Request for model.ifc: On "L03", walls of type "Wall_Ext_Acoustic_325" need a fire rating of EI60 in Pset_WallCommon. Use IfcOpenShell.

First a look at what the model holds.

```python
import ifcopenshell
import ifcopenshell.util.element

model = ifcopenshell.open("model.ifc")
print(model.schema)
storey = next(s for s in model.by_type("IfcBuildingStorey") if s.Name == "L03")
walls = [e for e in ifcopenshell.util.element.get_decomposition(storey) if e.is_a("IfcWall")]
seen = {}
for e in walls:
    element_type = ifcopenshell.util.element.get_type(e)
    key = (element_type.Name if element_type != e and element_type else None, ifcopenshell.util.element.get_pset(e, "Pset_WallCommon", "FireRating"))
    seen[key] = seen.get(key, 0) + 1
for (name, value), count in sorted(seen.items(), key=str):
    print(count, "x", name, "|", value)
```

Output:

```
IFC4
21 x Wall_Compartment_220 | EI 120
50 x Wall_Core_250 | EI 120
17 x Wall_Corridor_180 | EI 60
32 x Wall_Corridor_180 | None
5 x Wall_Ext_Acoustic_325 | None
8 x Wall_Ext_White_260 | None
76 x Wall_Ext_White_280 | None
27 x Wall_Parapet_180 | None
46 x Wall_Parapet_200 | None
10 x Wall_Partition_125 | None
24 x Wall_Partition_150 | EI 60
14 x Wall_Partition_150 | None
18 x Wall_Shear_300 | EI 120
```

```python
import ifcopenshell
import ifcopenshell.api.pset
import ifcopenshell.util.element

model = ifcopenshell.open("model.ifc")

storey = next(s for s in model.by_type("IfcBuildingStorey") if s.Name == "L03")
walls = [e for e in ifcopenshell.util.element.get_decomposition(storey) if e.is_a("IfcWall")]

count = 0
for e in walls:
    element_type = ifcopenshell.util.element.get_type(e)
    if element_type in (None, e) or element_type.Name != "Wall_Ext_Acoustic_325":
        continue
    # add_pset returns the element's existing set when there is one.
    pset = ifcopenshell.api.pset.add_pset(model, product=e, name="Pset_WallCommon")
    ifcopenshell.api.pset.edit_pset(model, pset=pset, properties={"FireRating": "EI60"})
    count += 1

print(count, "walls updated")

model.write("model-out.ifc")
```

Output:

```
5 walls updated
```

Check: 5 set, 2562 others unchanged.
